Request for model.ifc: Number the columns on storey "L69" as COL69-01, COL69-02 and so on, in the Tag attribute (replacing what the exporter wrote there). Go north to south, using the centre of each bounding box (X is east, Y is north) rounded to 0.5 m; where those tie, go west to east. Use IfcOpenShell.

First a look at what the model holds.

```python
import ifcopenshell
import ifcopenshell.util.element
import ifcopenshell.util.placement

model = ifcopenshell.open("model.ifc")
print(model.schema)
storey = next(s for s in model.by_type("IfcBuildingStorey") if s.Name == "L69")
columns = [e for e in ifcopenshell.util.element.get_decomposition(storey) if e.is_a("IfcColumn")]
for e in sorted(columns, key=lambda e: e.id()):
    origin = ifcopenshell.util.placement.get_local_placement(e.ObjectPlacement)[:3, 3]
    print(e.id(), e.Tag, e.Name, origin.round(2) + 0.0, sep=" | ")
```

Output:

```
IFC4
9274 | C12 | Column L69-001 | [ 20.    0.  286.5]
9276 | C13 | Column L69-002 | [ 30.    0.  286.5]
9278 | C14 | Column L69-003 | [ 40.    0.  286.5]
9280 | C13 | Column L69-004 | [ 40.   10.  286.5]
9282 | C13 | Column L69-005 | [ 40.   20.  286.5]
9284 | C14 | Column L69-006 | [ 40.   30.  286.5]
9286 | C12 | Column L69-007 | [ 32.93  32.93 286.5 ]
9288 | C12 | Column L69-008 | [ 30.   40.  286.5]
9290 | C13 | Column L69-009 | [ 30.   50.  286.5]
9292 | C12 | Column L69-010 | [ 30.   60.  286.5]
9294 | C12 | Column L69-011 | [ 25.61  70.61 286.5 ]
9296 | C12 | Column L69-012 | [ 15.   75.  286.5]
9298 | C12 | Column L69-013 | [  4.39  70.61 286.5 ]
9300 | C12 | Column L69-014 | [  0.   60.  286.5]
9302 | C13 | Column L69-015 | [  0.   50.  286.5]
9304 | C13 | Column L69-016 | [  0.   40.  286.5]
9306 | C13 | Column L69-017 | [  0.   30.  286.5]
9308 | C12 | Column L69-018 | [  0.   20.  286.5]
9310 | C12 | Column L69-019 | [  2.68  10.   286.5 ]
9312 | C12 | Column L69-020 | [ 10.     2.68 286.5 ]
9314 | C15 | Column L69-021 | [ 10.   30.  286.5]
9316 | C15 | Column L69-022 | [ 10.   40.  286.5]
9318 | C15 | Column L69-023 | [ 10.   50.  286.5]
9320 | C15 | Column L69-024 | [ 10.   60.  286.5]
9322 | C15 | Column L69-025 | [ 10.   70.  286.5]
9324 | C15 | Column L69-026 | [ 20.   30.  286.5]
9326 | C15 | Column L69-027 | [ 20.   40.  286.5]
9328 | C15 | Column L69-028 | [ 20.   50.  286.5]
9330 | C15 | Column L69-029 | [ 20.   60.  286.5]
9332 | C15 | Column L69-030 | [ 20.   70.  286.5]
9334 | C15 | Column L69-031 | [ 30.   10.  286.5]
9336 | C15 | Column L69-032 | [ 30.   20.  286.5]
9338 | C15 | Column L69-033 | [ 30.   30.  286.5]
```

```python
import ifcopenshell
import ifcopenshell.geom
import ifcopenshell.util.element
import ifcopenshell.util.shape

model = ifcopenshell.open("model.ifc")
settings = ifcopenshell.geom.settings()
settings.set("use-world-coords", True)


def centre(element):
    shape = ifcopenshell.geom.create_shape(settings, element)
    return ifcopenshell.util.shape.get_bbox_centroid(shape.geometry)


storey = next(s for s in model.by_type("IfcBuildingStorey") if s.Name == "L69")
columns = [e for e in ifcopenshell.util.element.get_decomposition(storey) if e.is_a("IfcColumn")]

# Insertion points can sit at a corner or the storey origin, so sort by the geometry (in metres).
centres = {e: centre(e) for e in columns}
columns.sort(key=lambda e: (-round(centres[e][1] / 0.5), centres[e][0]))

for i, e in enumerate(columns, start=1):
    number = f"COL69-{i:02d}"
    e.Tag = number
    print(e.id(), number)

model.write("model_edited.ifc")
```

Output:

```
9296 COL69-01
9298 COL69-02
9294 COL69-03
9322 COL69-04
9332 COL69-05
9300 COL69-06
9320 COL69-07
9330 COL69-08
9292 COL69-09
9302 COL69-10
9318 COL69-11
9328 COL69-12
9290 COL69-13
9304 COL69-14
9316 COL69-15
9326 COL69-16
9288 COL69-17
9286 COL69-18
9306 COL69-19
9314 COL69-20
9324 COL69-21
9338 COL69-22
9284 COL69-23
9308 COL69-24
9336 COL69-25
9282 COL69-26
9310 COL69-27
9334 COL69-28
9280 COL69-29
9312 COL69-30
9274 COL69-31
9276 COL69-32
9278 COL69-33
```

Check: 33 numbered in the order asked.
